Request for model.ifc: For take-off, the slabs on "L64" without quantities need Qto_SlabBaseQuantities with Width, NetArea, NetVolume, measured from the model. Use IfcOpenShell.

First a look at what the model holds.

```python
import ifcopenshell
import ifcopenshell.util.element
import ifcopenshell.util.unit

model = ifcopenshell.open("model.ifc")
print(model.schema)
for unit_type in ("LENGTHUNIT", "AREAUNIT", "VOLUMEUNIT"):
    print(unit_type, ifcopenshell.util.unit.calculate_unit_scale(model, unit_type))
storey = next(s for s in model.by_type("IfcBuildingStorey") if s.Name == "L64")
slabs = [e for e in ifcopenshell.util.element.get_decomposition(storey) if e.is_a("IfcSlab")]
for e in sorted(slabs, key=lambda e: e.id()):
    print(e.id(), e.is_a(), e.Name, list(ifcopenshell.util.element.get_psets(e, qtos_only=True)), sep=" | ")
```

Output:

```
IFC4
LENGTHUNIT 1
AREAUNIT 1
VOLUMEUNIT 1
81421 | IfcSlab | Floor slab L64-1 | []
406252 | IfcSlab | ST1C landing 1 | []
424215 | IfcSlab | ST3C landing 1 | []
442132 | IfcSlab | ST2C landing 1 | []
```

```python
import ifcopenshell
import ifcopenshell.api.pset
import ifcopenshell.geom
import ifcopenshell.util.element
import ifcopenshell.util.shape
import ifcopenshell.util.unit

model = ifcopenshell.open("model.ifc")
unit_scale = ifcopenshell.util.unit.calculate_unit_scale(model)
area_scale = ifcopenshell.util.unit.calculate_unit_scale(model, "AREAUNIT")
volume_scale = ifcopenshell.util.unit.calculate_unit_scale(model, "VOLUMEUNIT")
settings = ifcopenshell.geom.settings()

storey = next(s for s in model.by_type("IfcBuildingStorey") if s.Name == "L64")
slabs = [e for e in ifcopenshell.util.element.get_decomposition(storey) if e.is_a("IfcSlab")]

for e in sorted(slabs, key=lambda e: e.id()):
    if ifcopenshell.util.element.get_psets(e, qtos_only=True, should_inherit=False):
        continue
    # Geometry comes back in metres, in the element's own axes.
    shape = ifcopenshell.geom.create_shape(settings, e)
    values = {
        "Width": ifcopenshell.util.shape.get_z(shape.geometry) / unit_scale,
        "NetArea": ifcopenshell.util.shape.get_footprint_area(shape.geometry) / area_scale,
        "NetVolume": ifcopenshell.util.shape.get_volume(shape.geometry) / volume_scale,
    }
    qto = ifcopenshell.api.pset.add_qto(model, product=e, name="Qto_SlabBaseQuantities")
    ifcopenshell.api.pset.edit_qto(model, qto=qto, properties=values)
    print(e.id(), {k: round(v, 3) for k, v in values.items()})

model.write("model_edited.ifc")
```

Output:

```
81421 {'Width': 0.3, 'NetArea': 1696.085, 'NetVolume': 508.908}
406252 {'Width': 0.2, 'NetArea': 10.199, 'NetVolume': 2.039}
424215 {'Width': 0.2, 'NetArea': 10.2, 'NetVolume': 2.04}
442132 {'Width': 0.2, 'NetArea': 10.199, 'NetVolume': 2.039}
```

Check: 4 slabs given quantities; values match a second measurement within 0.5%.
